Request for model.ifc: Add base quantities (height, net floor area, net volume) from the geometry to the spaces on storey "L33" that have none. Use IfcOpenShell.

First a look at what the model holds.

```python
import ifcopenshell
import ifcopenshell.util.element
import ifcopenshell.util.unit

model = ifcopenshell.open("model.ifc")
print(model.schema)
for unit_type in ("LENGTHUNIT", "AREAUNIT", "VOLUMEUNIT"):
    print(unit_type, ifcopenshell.util.unit.calculate_unit_scale(model, unit_type))
storey = next(s for s in model.by_type("IfcBuildingStorey") if s.Name == "L33")
spaces = [e for e in ifcopenshell.util.element.get_decomposition(storey) if e.is_a("IfcSpace")]
for e in sorted(spaces, key=lambda e: e.id()):
    print(e.id(), e.is_a(), e.Name, list(ifcopenshell.util.element.get_psets(e, qtos_only=True)), sep=" | ")
```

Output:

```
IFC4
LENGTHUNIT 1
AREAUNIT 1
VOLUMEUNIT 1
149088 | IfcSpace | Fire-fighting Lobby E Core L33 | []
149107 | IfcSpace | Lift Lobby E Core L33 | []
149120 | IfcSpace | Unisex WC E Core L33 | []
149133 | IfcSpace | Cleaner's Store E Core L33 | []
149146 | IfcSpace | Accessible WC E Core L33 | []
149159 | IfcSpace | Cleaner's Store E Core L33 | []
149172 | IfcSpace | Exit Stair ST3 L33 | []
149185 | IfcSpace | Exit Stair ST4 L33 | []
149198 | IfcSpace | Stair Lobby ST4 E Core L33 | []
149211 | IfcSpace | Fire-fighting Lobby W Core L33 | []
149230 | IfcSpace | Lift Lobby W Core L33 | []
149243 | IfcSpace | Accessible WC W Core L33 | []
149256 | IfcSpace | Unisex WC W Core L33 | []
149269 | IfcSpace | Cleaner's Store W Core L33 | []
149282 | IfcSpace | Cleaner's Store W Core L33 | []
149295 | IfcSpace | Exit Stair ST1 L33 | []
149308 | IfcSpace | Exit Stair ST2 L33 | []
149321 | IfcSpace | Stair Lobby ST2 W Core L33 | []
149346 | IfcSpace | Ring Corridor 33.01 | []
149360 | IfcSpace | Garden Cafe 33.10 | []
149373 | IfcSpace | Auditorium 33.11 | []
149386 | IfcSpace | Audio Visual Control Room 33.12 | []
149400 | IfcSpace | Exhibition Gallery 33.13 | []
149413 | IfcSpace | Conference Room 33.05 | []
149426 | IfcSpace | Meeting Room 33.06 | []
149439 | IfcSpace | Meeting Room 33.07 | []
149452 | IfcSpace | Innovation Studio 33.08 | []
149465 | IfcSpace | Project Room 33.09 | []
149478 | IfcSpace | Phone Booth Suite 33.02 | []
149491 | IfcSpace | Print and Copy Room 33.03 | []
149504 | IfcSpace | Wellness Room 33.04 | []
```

```python
import ifcopenshell
import ifcopenshell.api.pset
import ifcopenshell.geom
import ifcopenshell.util.element
import ifcopenshell.util.shape
import ifcopenshell.util.unit

model = ifcopenshell.open("model.ifc")
unit_scale = ifcopenshell.util.unit.calculate_unit_scale(model)
area_scale = ifcopenshell.util.unit.calculate_unit_scale(model, "AREAUNIT")
volume_scale = ifcopenshell.util.unit.calculate_unit_scale(model, "VOLUMEUNIT")
settings = ifcopenshell.geom.settings()

storey = next(s for s in model.by_type("IfcBuildingStorey") if s.Name == "L33")
spaces = [e for e in ifcopenshell.util.element.get_decomposition(storey) if e.is_a("IfcSpace")]

for e in sorted(spaces, key=lambda e: e.id()):
    if ifcopenshell.util.element.get_psets(e, qtos_only=True, should_inherit=False):
        continue
    # Geometry comes back in metres, in the element's own axes.
    shape = ifcopenshell.geom.create_shape(settings, e)
    values = {
        "Height": ifcopenshell.util.shape.get_z(shape.geometry) / unit_scale,
        "NetFloorArea": ifcopenshell.util.shape.get_footprint_area(shape.geometry) / area_scale,
        "NetVolume": ifcopenshell.util.shape.get_volume(shape.geometry) / volume_scale,
    }
    qto = ifcopenshell.api.pset.add_qto(model, product=e, name="Qto_SpaceBaseQuantities")
    ifcopenshell.api.pset.edit_qto(model, qto=qto, properties=values)
    print(e.id(), {k: round(v, 3) for k, v in values.items()})

model.write("model_updated.ifc")
```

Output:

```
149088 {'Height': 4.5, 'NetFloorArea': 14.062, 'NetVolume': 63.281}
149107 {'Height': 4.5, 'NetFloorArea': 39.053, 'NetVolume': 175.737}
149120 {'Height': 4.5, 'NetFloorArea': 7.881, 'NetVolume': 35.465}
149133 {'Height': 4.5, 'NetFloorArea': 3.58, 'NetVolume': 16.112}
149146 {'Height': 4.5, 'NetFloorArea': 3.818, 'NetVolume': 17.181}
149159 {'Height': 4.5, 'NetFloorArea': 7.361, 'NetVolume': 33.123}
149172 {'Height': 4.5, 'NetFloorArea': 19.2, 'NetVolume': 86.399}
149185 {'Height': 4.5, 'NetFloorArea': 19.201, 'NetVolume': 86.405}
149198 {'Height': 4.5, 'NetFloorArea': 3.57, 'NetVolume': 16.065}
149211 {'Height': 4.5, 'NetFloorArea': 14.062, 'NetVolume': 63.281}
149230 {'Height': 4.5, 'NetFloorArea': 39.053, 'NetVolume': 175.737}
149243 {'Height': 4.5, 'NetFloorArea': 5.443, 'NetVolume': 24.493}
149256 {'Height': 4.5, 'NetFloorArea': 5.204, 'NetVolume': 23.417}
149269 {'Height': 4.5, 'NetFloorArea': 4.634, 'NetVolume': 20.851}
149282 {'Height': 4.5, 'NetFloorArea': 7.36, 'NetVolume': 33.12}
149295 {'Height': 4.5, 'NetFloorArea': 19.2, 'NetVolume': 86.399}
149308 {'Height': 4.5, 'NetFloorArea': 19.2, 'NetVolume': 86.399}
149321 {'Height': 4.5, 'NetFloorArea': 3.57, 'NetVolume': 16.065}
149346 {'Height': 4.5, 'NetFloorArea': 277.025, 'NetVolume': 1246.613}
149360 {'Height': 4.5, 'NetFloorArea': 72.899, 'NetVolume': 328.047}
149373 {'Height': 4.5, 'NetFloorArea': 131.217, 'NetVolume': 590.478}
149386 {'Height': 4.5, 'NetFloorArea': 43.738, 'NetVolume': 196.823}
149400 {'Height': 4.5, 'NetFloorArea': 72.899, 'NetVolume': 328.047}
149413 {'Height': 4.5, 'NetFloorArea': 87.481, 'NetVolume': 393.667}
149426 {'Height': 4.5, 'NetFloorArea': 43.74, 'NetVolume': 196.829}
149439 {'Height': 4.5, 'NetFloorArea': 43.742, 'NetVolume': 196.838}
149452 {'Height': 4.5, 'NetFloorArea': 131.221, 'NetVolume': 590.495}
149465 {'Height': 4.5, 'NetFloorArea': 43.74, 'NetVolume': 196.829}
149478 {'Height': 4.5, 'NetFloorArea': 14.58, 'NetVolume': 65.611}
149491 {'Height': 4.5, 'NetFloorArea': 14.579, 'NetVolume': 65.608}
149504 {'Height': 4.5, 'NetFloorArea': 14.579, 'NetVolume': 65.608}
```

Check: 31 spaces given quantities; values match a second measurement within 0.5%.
